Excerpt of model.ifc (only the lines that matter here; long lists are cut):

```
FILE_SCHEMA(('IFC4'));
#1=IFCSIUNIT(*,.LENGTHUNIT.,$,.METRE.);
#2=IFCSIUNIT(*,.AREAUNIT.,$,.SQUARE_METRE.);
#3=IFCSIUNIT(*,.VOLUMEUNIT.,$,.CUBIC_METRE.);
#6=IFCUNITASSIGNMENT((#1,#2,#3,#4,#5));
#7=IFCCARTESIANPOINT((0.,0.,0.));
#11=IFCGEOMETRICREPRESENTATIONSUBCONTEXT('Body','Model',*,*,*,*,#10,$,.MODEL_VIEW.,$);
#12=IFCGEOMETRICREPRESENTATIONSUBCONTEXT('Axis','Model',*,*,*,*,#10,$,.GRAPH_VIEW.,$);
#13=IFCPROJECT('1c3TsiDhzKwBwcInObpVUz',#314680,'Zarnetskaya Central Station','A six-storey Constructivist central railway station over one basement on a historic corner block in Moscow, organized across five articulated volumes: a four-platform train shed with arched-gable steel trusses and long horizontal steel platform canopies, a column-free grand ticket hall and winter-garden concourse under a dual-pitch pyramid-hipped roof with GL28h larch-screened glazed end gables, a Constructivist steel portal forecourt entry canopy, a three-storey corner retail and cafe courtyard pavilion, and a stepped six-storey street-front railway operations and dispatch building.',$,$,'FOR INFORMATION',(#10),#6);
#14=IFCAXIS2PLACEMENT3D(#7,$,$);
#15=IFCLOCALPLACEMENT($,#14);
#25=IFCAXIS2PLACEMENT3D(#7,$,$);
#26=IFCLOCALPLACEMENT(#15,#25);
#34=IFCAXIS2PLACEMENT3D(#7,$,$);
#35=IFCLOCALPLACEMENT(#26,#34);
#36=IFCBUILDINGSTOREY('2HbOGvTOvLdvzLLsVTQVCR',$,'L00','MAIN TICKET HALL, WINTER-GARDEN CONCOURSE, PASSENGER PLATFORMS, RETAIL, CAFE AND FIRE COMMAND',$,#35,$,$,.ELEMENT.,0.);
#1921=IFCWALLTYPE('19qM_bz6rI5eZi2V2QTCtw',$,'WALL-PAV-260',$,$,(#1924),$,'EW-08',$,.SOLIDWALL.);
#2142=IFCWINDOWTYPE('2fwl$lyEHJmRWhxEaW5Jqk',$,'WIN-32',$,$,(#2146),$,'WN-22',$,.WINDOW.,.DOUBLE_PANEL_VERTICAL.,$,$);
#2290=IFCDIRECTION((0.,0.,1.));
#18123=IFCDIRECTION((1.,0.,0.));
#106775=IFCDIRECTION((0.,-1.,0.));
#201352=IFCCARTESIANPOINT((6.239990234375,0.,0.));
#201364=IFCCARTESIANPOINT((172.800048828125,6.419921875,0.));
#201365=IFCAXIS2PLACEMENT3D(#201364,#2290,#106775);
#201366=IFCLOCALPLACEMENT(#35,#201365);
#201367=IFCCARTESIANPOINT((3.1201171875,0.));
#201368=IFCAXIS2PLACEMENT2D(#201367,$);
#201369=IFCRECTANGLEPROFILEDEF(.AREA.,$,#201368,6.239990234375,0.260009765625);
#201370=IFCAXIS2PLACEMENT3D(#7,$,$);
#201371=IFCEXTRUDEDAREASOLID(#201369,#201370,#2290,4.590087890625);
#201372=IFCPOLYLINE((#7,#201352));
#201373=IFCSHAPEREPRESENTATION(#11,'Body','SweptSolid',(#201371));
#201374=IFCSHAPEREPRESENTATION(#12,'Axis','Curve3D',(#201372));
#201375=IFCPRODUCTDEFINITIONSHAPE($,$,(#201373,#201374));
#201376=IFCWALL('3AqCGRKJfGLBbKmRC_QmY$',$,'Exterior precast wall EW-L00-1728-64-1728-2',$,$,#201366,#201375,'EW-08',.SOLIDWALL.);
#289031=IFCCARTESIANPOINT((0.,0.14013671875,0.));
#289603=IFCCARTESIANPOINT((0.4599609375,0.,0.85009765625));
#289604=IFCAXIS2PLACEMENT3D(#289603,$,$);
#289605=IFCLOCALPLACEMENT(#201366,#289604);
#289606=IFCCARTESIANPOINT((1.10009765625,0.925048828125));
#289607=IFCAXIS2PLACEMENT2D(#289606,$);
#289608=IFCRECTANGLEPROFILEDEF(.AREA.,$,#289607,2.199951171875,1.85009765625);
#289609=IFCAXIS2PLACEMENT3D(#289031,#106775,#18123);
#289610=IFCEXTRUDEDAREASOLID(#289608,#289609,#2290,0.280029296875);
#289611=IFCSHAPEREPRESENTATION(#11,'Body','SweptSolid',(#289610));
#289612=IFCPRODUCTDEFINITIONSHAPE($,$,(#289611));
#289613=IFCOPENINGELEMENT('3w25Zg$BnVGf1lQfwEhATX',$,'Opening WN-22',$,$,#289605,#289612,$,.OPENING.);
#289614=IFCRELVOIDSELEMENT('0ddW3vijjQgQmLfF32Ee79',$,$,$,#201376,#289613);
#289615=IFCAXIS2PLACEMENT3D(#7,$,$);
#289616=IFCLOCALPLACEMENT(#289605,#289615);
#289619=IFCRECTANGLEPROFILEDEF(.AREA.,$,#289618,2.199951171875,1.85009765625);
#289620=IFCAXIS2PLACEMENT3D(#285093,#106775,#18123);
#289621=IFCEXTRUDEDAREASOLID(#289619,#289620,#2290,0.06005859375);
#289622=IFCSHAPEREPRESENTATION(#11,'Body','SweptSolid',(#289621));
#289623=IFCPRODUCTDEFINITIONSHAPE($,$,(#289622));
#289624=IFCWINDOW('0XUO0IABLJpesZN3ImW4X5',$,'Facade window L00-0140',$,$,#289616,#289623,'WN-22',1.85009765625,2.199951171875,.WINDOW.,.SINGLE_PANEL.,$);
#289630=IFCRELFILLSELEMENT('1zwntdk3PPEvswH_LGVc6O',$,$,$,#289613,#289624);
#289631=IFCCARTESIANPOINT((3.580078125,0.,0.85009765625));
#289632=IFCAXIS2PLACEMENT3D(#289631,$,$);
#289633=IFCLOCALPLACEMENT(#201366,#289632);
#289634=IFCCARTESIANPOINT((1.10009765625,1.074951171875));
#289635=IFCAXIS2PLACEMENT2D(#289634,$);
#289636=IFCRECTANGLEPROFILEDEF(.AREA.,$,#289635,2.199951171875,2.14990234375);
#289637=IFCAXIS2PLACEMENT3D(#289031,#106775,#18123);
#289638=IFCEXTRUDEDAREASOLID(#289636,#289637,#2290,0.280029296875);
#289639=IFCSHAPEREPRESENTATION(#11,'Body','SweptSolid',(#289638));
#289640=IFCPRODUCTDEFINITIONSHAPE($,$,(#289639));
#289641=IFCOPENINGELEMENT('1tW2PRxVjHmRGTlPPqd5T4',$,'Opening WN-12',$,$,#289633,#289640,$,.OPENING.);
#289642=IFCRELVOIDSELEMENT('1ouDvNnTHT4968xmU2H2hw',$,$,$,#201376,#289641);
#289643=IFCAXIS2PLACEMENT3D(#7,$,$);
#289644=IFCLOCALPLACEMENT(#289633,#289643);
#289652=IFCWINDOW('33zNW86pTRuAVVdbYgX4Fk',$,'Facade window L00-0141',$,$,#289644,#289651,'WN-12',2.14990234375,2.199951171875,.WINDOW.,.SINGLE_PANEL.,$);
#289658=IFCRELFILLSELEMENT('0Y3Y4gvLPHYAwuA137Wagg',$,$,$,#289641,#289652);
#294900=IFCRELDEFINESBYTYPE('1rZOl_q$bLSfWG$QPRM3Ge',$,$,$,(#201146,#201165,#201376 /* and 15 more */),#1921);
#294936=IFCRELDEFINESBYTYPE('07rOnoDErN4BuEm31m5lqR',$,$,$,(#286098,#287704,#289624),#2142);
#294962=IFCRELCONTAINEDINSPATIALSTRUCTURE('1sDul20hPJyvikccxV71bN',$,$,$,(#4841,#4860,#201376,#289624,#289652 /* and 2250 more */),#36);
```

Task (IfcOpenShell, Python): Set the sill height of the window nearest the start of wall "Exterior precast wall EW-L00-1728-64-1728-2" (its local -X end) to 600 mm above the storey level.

```python
import numpy as np
import ifcopenshell
import ifcopenshell.api.geometry
import ifcopenshell.geom
import ifcopenshell.util.element
import ifcopenshell.util.placement
import ifcopenshell.util.shape
import ifcopenshell.util.unit

model = ifcopenshell.open("model.ifc")
unit_scale = ifcopenshell.util.unit.calculate_unit_scale(model)

window = model.by_guid("0XUO0IABLJpesZN3ImW4X5")
opening = window.FillsVoids[0].RelatingOpeningElement
storey = ifcopenshell.util.element.get_container(window, ifc_class="IfcBuildingStorey")
level = ifcopenshell.util.placement.get_local_placement(storey.ObjectPlacement)[2, 3]

# The opening's origin need not be at the sill, so measure its lowest point.
shape = ifcopenshell.geom.create_shape(ifcopenshell.geom.settings(), opening)
bottom = ifcopenshell.util.shape.get_shape_bottom_elevation(shape, shape.geometry) / unit_scale
dz = level + 0.6 / unit_scale - bottom

shift = np.array([0.0, 0.0, dz])
# The window is placed relative to its opening, so it follows when the opening moves.
matrix = ifcopenshell.util.placement.get_local_placement(opening.ObjectPlacement)
matrix[:3, 3] += shift
ifcopenshell.api.geometry.edit_object_placement(
    model, product=opening, matrix=matrix, is_si=False, should_transform_children=True
)

print(f"moved by {dz * unit_scale:+.3f} m")

model.write("model-out.ifc")
```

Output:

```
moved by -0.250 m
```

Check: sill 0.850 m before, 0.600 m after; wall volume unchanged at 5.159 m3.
